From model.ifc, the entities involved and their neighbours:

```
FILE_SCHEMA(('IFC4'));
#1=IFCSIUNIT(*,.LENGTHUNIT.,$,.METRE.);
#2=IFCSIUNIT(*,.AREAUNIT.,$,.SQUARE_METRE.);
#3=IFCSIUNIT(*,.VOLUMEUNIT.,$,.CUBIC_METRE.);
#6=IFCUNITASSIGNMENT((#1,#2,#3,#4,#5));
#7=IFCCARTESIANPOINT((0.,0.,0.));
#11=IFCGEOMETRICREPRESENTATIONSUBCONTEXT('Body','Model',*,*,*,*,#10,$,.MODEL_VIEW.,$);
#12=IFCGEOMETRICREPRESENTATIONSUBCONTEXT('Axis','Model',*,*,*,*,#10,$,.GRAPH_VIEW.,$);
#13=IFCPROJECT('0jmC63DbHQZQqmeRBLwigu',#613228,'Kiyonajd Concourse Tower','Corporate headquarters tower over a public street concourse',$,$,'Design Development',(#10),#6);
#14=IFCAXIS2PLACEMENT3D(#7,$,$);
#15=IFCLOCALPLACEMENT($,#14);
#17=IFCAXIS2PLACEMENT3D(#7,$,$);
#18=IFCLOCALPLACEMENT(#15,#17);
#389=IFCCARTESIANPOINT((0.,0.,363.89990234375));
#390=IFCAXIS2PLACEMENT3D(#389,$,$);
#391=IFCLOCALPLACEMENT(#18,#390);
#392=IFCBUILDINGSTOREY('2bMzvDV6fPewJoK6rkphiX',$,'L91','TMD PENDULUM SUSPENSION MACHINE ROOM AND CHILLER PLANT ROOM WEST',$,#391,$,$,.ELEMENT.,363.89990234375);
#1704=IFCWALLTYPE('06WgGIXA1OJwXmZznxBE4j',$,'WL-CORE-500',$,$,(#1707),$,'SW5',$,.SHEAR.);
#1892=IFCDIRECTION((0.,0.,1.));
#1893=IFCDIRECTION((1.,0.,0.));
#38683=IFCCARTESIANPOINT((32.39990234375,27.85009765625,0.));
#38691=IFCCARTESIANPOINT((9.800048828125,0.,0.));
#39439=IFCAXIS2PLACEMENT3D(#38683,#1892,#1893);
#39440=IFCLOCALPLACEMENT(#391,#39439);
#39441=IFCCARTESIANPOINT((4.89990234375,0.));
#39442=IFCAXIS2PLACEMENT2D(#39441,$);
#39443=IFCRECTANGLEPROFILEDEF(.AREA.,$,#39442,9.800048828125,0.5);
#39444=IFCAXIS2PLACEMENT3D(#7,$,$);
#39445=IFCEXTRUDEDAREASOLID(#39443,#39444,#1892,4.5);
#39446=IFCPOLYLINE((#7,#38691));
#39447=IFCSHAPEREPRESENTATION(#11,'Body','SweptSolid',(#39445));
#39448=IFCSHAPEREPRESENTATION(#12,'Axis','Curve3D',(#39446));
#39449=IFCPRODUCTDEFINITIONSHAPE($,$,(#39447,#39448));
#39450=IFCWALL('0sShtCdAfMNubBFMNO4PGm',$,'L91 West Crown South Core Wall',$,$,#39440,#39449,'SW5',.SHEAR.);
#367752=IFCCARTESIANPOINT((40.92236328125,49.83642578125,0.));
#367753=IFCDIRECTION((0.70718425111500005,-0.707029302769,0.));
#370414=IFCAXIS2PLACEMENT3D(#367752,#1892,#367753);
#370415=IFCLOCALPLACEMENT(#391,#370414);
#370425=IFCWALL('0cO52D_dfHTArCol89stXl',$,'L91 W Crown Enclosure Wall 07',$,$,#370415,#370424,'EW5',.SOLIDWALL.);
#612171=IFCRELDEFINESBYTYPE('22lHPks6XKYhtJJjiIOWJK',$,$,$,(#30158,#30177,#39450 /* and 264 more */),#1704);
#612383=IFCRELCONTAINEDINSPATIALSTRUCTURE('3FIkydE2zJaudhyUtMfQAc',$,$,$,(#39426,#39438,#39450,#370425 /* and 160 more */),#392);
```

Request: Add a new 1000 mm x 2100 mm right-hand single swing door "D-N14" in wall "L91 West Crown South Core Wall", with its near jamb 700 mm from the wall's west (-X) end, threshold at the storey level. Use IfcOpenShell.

```python
import numpy as np
import ifcopenshell
import ifcopenshell.api.feature
import ifcopenshell.api.geometry
import ifcopenshell.api.root
import ifcopenshell.api.spatial
import ifcopenshell.geom
import ifcopenshell.util.element
import ifcopenshell.util.placement
import ifcopenshell.util.representation
import ifcopenshell.util.shape
import ifcopenshell.util.unit

model = ifcopenshell.open("model.ifc")
unit_scale = ifcopenshell.util.unit.calculate_unit_scale(model)
settings = ifcopenshell.geom.settings()


def volume(element):
    """Net volume in cubic metres, openings subtracted."""
    shape = ifcopenshell.geom.create_shape(settings, element)
    return ifcopenshell.util.shape.get_volume(shape.geometry)


wall = model.by_id(39450)
storey = ifcopenshell.util.element.get_container(wall, ifc_class="IfcBuildingStorey")
context = ifcopenshell.util.representation.get_context(model, "Model", "Body", "MODEL_VIEW")
before = volume(wall)

width, height, from_end, sill = 1, 2.1, 0.7, 0.0  # metres

# The wall runs along its own X axis, and the end named is its -X end.
wall_shape = ifcopenshell.geom.create_shape(settings, wall)
x, y, z = ifcopenshell.util.shape.get_vertices(wall_shape.geometry).T
start = x.min() + from_end
face, thickness = float(y.min()), float(y.max() - y.min())
wall_matrix = ifcopenshell.util.placement.get_local_placement(wall.ObjectPlacement)
level = ifcopenshell.util.placement.get_local_placement(storey.ObjectPlacement)[2, 3]


def in_wall(x, y):
    """Placement at x, y metres in the wall's axes, at sill height."""
    matrix = wall_matrix.copy()
    matrix[:, 3] = wall_matrix @ np.array([x / unit_scale, y / unit_scale, 0.0, 1.0])
    matrix[2, 3] = level + sill / unit_scale
    return matrix


# Opening: a box that overshoots both wall faces by 50 mm.
opening = ifcopenshell.api.root.create_entity(model, ifc_class="IfcOpeningElement", predefined_type="OPENING")
box = ifcopenshell.api.geometry.add_wall_representation(
    model, context=context, length=width, height=height, thickness=thickness + 0.1
)
ifcopenshell.api.geometry.assign_representation(model, product=opening, representation=box)
ifcopenshell.api.geometry.edit_object_placement(model, product=opening, matrix=in_wall(start, face - 0.05), is_si=False)
ifcopenshell.api.feature.add_feature(model, feature=opening, element=wall)

door = ifcopenshell.api.root.create_entity(model, ifc_class="IfcDoor", name="D-N14", predefined_type="DOOR")
door.OverallWidth, door.OverallHeight = width / unit_scale, height / unit_scale
door.OperationType = "SINGLE_SWING_RIGHT"
body = ifcopenshell.api.geometry.add_door_representation(
    model,
    context=context,
    overall_width=door.OverallWidth,
    overall_height=door.OverallHeight,
    operation_type="SINGLE_SWING_RIGHT",
    lining_properties={"LiningDepth": thickness / unit_scale, "ThresholdDepth": thickness / unit_scale},
)
ifcopenshell.api.geometry.assign_representation(model, product=door, representation=body)
ifcopenshell.api.spatial.assign_container(model, products=[door], relating_structure=storey)
ifcopenshell.api.feature.add_filling(model, opening=opening, element=door)

# The lining spans the wall, so the door starts at the wall face.
ifcopenshell.api.geometry.edit_object_placement(model, product=door, matrix=in_wall(start, face), is_si=False)

after = volume(wall)

print(f"wall volume {before:.3f} -> {after:.3f} m3")

model.write("model-out.ifc")
```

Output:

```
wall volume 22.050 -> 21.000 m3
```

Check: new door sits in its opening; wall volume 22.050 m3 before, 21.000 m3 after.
